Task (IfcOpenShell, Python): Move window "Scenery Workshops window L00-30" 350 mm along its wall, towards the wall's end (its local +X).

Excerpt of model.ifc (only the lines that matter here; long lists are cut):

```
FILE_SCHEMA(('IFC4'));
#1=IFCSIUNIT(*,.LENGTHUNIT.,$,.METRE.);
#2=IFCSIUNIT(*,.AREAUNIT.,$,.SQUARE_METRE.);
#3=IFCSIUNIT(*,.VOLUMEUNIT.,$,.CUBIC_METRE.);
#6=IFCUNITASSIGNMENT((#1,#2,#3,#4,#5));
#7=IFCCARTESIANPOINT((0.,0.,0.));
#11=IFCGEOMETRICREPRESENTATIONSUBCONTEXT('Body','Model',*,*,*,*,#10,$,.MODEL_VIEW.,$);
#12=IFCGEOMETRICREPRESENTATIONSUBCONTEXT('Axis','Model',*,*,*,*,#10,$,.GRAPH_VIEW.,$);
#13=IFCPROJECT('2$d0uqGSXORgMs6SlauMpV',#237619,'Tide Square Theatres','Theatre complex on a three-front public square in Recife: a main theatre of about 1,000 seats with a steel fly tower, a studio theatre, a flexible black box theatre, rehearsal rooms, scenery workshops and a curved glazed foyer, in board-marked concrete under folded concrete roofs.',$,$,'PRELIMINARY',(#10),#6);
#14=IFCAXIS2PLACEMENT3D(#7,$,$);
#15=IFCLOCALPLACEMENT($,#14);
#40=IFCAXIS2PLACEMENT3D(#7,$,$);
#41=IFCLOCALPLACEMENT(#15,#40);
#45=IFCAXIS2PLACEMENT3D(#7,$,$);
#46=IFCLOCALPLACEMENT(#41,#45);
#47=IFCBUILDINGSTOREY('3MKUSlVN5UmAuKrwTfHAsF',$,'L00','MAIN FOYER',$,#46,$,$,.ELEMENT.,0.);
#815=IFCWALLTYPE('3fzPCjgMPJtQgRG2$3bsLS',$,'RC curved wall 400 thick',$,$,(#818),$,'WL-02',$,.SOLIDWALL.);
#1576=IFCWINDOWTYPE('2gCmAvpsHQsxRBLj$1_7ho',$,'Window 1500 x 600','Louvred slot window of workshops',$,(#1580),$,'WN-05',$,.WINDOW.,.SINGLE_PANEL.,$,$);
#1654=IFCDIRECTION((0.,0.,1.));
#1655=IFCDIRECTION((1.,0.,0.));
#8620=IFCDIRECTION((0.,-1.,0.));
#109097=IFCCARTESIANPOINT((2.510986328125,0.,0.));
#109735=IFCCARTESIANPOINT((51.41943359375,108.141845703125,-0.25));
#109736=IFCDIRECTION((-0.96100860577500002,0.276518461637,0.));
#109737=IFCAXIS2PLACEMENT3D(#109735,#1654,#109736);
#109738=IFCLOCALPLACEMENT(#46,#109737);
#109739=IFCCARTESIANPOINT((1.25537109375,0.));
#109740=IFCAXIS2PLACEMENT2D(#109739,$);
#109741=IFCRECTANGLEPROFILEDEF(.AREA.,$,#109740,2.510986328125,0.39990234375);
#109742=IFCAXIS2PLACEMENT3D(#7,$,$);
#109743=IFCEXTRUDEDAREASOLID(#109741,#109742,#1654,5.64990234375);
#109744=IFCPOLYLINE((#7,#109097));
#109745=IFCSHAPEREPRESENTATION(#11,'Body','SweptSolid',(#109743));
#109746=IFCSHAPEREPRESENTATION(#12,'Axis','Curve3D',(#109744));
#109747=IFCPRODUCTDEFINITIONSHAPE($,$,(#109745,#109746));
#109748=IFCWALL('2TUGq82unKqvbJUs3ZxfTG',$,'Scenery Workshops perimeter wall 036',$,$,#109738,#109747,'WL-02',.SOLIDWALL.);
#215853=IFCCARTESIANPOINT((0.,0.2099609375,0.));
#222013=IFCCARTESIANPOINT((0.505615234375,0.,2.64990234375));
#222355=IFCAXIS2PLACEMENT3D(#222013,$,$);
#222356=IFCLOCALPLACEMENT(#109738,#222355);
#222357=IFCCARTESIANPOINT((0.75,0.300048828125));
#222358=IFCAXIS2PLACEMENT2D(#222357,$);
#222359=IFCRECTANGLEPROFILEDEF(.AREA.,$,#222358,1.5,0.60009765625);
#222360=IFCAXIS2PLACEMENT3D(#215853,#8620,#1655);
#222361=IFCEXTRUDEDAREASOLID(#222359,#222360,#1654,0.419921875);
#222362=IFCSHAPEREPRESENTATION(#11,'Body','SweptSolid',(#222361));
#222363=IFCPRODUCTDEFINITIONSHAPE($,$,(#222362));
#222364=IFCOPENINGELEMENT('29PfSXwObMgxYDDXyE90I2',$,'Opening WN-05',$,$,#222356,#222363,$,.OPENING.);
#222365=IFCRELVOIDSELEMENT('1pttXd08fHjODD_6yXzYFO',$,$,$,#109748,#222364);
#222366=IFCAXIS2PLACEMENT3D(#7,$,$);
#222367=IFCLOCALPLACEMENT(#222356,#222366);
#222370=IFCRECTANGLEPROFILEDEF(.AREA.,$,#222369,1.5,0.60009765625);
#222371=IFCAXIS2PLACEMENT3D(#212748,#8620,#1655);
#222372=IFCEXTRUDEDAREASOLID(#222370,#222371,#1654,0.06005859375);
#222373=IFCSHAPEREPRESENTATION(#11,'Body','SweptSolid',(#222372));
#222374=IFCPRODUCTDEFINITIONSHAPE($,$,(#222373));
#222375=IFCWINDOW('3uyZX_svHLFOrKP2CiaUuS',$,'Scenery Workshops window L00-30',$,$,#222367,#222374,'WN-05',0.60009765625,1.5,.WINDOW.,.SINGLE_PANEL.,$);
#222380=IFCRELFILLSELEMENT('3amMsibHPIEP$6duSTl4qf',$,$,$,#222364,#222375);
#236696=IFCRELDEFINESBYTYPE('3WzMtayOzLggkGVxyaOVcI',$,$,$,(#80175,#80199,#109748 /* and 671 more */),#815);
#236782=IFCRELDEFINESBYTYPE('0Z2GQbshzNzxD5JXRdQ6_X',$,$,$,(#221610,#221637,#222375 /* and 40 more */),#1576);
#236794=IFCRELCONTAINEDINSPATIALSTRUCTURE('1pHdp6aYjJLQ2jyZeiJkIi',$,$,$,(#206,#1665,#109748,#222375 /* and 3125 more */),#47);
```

```python
import ifcopenshell
import ifcopenshell.api.geometry
import ifcopenshell.util.placement

model = ifcopenshell.open("model.ifc")

window = model.by_id(222375)
opening = window.FillsVoids[0].RelatingOpeningElement
wall = opening.VoidsElements[0].RelatingBuildingElement

wall_matrix = ifcopenshell.util.placement.get_local_placement(wall.ObjectPlacement)
shift = wall_matrix[:3, 0] * 0.35
before = ifcopenshell.util.placement.get_local_placement(window.ObjectPlacement)[:3, 3].copy()

# The window is placed relative to its opening, so it follows when the opening moves.
matrix = ifcopenshell.util.placement.get_local_placement(opening.ObjectPlacement)
matrix[:3, 3] += shift
ifcopenshell.api.geometry.edit_object_placement(
    model, product=opening, matrix=matrix, is_si=False, should_transform_children=True
)

after = ifcopenshell.util.placement.get_local_placement(window.ObjectPlacement)[:3, 3]
print("window moved by", (after - before).round(3) + 0.0)

model.write("model_v2.ifc")
```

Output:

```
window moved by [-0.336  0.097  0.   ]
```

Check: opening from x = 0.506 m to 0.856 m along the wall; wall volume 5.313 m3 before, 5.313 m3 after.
